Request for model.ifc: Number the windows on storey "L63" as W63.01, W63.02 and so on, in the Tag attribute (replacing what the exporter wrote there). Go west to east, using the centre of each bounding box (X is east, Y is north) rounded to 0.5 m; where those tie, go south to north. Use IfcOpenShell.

First a look at what the model holds.

```python
import ifcopenshell
import ifcopenshell.util.element
import ifcopenshell.util.placement

model = ifcopenshell.open("model.ifc")
print(model.schema)
storey = next(s for s in model.by_type("IfcBuildingStorey") if s.Name == "L63")
windows = [e for e in ifcopenshell.util.element.get_decomposition(storey) if e.is_a("IfcWindow")]
for e in sorted(windows, key=lambda e: e.id()):
    origin = ifcopenshell.util.placement.get_local_placement(e.ObjectPlacement)[:3, 3]
    print(e.id(), e.Tag, e.Name, origin.round(2) + 0.0, sep=" | ")
```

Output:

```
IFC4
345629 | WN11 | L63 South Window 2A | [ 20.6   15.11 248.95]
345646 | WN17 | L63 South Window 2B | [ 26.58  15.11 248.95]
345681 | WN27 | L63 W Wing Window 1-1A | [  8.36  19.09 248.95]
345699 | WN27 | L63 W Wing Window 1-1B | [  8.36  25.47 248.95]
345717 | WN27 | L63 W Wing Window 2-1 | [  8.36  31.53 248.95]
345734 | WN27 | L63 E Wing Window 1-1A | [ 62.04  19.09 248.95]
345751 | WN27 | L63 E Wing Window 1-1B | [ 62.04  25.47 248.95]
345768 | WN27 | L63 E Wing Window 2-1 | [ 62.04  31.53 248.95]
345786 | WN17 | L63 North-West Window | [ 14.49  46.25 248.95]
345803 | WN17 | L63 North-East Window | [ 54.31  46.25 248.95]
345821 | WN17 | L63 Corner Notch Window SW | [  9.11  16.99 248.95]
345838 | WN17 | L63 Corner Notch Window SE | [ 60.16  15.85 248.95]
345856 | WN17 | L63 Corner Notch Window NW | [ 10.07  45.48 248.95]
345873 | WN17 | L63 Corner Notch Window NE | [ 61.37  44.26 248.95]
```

```python
import ifcopenshell
import ifcopenshell.geom
import ifcopenshell.util.element
import ifcopenshell.util.shape

model = ifcopenshell.open("model.ifc")
settings = ifcopenshell.geom.settings()
settings.set("use-world-coords", True)


def centre(element):
    shape = ifcopenshell.geom.create_shape(settings, element)
    return ifcopenshell.util.shape.get_bbox_centroid(shape.geometry)


storey = next(s for s in model.by_type("IfcBuildingStorey") if s.Name == "L63")
windows = [e for e in ifcopenshell.util.element.get_decomposition(storey) if e.is_a("IfcWindow")]

# Insertion points can sit at a corner or the storey origin, so sort by the geometry (in metres).
centres = {e: centre(e) for e in windows}
windows.sort(key=lambda e: (round(centres[e][0] / 0.5), centres[e][1]))

for i, e in enumerate(windows, start=1):
    number = f"W63.{i:02d}"
    e.Tag = number
    print(e.id(), number)

model.write("model_rev.ifc")
```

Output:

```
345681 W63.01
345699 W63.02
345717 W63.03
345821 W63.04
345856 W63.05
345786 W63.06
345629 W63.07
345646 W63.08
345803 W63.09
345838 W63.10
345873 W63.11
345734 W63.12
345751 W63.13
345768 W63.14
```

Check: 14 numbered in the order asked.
